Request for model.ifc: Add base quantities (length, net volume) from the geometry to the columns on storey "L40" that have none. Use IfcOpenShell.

First a look at what the model holds.

```python
import ifcopenshell
import ifcopenshell.util.element
import ifcopenshell.util.unit

model = ifcopenshell.open("model.ifc")
print(model.schema)
for unit_type in ("LENGTHUNIT", "AREAUNIT", "VOLUMEUNIT"):
    print(unit_type, ifcopenshell.util.unit.calculate_unit_scale(model, unit_type))
storey = next(s for s in model.by_type("IfcBuildingStorey") if s.Name == "L40")
columns = [e for e in ifcopenshell.util.element.get_decomposition(storey) if e.is_a("IfcColumn")]
for e in sorted(columns, key=lambda e: e.id()):
    print(e.id(), e.is_a(), e.Name, list(ifcopenshell.util.element.get_psets(e, qtos_only=True)), sep=" | ")
```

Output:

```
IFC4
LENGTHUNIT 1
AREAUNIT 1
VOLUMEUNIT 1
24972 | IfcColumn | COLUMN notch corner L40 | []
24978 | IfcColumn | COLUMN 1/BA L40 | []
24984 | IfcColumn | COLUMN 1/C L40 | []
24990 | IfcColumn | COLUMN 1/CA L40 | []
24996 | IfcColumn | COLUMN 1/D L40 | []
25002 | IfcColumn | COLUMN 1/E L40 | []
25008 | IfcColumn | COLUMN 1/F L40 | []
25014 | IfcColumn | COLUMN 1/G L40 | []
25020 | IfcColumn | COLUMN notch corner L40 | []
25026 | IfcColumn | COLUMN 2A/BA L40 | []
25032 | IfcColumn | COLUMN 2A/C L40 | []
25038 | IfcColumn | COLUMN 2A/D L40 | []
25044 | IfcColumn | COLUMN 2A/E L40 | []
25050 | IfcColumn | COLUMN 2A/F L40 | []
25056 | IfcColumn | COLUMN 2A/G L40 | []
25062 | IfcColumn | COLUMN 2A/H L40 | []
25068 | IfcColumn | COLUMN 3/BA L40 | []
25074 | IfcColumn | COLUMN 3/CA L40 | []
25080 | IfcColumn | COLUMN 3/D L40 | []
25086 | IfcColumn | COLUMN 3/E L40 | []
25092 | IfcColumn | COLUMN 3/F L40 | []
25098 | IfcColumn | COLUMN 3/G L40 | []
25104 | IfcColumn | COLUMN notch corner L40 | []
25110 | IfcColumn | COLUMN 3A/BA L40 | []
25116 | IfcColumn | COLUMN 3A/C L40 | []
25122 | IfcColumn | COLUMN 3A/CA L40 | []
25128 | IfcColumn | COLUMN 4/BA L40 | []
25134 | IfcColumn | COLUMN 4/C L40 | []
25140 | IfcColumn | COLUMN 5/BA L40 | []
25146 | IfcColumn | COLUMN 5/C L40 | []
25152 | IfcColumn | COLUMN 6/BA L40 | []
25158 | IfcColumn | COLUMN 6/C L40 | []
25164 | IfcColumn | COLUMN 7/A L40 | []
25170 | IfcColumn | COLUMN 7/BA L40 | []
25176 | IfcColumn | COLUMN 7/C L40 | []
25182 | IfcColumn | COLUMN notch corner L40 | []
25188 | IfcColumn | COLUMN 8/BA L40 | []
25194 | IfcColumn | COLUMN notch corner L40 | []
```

```python
import ifcopenshell
import ifcopenshell.api.pset
import ifcopenshell.geom
import ifcopenshell.util.element
import ifcopenshell.util.shape
import ifcopenshell.util.unit

model = ifcopenshell.open("model.ifc")
unit_scale = ifcopenshell.util.unit.calculate_unit_scale(model)
volume_scale = ifcopenshell.util.unit.calculate_unit_scale(model, "VOLUMEUNIT")
settings = ifcopenshell.geom.settings()

storey = next(s for s in model.by_type("IfcBuildingStorey") if s.Name == "L40")
columns = [e for e in ifcopenshell.util.element.get_decomposition(storey) if e.is_a("IfcColumn")]

for e in sorted(columns, key=lambda e: e.id()):
    if ifcopenshell.util.element.get_psets(e, qtos_only=True, should_inherit=False):
        continue
    # Geometry comes back in metres, in the element's own axes.
    shape = ifcopenshell.geom.create_shape(settings, e)
    values = {
        "Length": ifcopenshell.util.shape.get_z(shape.geometry) / unit_scale,
        "NetVolume": ifcopenshell.util.shape.get_volume(shape.geometry) / volume_scale,
    }
    qto = ifcopenshell.api.pset.add_qto(model, product=e, name="Qto_ColumnBaseQuantities")
    ifcopenshell.api.pset.edit_qto(model, qto=qto, properties=values)
    print(e.id(), {k: round(v, 3) for k, v in values.items()})

model.write("model_updated.ifc")
```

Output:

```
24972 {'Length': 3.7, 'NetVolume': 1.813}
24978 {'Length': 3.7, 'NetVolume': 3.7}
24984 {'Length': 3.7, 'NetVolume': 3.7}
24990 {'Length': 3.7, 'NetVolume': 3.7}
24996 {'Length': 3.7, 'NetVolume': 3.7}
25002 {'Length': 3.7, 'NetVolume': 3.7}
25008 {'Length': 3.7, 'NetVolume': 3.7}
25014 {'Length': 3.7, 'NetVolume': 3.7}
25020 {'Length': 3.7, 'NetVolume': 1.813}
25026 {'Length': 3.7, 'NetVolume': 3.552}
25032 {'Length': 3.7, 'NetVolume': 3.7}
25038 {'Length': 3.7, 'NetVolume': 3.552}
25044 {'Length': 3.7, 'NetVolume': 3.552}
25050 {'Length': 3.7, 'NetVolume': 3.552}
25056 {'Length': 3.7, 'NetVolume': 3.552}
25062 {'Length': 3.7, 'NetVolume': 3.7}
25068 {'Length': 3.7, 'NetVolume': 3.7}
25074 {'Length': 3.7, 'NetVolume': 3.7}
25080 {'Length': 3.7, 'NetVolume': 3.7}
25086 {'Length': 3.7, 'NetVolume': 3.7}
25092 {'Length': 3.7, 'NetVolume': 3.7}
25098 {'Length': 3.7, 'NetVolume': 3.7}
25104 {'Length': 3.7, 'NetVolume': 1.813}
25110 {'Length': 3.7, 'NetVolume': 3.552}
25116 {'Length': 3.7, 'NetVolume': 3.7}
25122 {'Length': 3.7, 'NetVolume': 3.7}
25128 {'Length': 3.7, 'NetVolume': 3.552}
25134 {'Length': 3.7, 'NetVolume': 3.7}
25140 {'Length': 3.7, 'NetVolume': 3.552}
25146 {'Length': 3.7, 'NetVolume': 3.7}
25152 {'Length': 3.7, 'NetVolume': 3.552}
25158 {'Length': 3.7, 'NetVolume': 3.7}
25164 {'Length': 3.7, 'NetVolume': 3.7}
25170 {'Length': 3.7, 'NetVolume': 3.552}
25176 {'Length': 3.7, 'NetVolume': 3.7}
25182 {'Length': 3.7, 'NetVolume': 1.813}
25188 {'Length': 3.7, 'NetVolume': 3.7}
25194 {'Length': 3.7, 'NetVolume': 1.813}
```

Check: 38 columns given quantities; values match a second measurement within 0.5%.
